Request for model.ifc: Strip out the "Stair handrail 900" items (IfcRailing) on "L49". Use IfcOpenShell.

First a look at what the model holds.

```python
import ifcopenshell
import ifcopenshell.util.element

model = ifcopenshell.open("model.ifc")
print(model.schema)
storey = next(s for s in model.by_type("IfcBuildingStorey") if s.Name == "L49")
railings = [e for e in ifcopenshell.util.element.get_decomposition(storey) if e.is_a("IfcRailing")]
seen = {}
for e in railings:
    element_type = ifcopenshell.util.element.get_type(e)
    name = element_type.Name if element_type not in (None, e) else None
    seen[name] = seen.get(name, 0) + 1
for name, count in sorted(seen.items(), key=str):
    print(count, "x", name)
```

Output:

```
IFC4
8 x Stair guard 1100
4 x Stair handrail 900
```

```python
import ifcopenshell
import ifcopenshell.api.root
import ifcopenshell.util.element

model = ifcopenshell.open("model.ifc")

storey = next(s for s in model.by_type("IfcBuildingStorey") if s.Name == "L49")
railings = [e for e in ifcopenshell.util.element.get_decomposition(storey) if e.is_a("IfcRailing")]
targets = [e for e in railings if (t := ifcopenshell.util.element.get_type(e)) not in (None, e) and t.Name == "Stair handrail 900"]

for e in targets:
    ifcopenshell.api.root.remove_product(model, product=e)
print(len(targets), "removed")

model.write("model_edited.ifc")
```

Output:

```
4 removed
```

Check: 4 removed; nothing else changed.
